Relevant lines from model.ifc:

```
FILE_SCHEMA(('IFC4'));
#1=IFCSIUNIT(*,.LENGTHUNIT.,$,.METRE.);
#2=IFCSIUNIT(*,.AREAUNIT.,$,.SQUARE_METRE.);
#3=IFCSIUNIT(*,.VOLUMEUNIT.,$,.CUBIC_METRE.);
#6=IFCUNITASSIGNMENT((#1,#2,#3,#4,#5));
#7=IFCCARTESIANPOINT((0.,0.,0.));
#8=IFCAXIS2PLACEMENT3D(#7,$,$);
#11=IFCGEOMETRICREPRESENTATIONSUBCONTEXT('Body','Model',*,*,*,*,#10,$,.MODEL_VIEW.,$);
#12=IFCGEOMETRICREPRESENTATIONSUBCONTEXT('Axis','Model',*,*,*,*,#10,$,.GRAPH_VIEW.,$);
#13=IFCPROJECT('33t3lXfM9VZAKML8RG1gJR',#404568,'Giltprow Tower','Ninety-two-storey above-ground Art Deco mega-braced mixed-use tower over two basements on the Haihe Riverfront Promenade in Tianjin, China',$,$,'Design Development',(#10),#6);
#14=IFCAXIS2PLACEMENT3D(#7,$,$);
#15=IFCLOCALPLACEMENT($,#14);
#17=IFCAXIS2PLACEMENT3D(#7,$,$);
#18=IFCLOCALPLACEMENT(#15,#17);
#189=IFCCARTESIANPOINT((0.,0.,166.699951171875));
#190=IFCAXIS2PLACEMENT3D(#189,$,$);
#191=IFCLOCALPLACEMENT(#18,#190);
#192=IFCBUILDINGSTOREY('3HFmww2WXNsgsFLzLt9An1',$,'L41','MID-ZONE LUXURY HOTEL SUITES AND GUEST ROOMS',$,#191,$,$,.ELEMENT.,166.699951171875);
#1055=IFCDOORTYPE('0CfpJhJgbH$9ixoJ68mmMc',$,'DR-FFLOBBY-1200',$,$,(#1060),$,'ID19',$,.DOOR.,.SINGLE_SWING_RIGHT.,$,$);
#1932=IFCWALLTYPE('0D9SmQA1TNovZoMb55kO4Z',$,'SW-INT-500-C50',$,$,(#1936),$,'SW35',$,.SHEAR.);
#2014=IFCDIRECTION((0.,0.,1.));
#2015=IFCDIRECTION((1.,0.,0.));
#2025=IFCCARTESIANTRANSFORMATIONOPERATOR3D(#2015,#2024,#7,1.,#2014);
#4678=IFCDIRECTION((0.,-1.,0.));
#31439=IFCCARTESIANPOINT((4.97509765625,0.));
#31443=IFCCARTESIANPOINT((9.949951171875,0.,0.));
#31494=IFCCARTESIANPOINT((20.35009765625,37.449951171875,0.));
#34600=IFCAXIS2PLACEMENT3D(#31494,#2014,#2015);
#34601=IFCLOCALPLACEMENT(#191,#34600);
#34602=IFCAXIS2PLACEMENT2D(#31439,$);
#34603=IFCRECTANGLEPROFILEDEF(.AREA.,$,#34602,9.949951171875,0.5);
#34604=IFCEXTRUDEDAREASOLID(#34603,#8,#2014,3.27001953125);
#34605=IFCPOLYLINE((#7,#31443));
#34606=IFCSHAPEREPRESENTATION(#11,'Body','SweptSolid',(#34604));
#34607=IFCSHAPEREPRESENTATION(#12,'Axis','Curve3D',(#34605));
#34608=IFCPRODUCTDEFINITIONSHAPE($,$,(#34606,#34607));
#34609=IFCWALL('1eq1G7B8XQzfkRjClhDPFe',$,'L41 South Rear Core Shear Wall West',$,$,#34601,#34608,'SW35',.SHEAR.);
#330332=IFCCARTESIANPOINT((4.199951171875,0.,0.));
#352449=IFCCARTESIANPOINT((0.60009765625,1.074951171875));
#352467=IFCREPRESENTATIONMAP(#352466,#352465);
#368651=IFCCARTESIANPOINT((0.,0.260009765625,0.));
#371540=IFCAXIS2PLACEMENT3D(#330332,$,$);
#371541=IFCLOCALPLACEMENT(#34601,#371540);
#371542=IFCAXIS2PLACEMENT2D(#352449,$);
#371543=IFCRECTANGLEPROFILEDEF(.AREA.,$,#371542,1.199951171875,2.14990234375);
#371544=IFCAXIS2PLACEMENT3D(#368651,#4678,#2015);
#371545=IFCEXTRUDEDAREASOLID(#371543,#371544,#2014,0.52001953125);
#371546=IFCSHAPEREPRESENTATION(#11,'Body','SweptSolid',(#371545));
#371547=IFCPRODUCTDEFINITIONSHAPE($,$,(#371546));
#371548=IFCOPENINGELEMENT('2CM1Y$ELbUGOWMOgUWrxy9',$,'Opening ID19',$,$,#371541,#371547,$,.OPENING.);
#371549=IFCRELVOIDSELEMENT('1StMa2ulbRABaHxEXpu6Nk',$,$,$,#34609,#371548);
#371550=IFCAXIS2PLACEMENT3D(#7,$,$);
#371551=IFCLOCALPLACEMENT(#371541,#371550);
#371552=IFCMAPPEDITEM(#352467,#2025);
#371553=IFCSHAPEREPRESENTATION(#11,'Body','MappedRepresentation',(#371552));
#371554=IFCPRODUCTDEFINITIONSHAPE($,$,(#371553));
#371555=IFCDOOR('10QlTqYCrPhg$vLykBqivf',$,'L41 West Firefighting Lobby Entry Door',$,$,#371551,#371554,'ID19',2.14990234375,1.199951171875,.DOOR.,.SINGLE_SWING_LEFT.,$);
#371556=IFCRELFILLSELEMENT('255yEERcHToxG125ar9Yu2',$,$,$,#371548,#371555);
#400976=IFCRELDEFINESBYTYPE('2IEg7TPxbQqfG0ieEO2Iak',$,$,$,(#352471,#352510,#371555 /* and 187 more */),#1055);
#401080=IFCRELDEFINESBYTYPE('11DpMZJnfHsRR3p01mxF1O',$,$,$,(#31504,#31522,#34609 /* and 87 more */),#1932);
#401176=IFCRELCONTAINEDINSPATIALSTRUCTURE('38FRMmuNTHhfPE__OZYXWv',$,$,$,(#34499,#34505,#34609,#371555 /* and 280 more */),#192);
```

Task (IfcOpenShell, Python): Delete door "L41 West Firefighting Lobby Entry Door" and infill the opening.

```python
import ifcopenshell
import ifcopenshell.api.feature
import ifcopenshell.api.root
import ifcopenshell.geom
import ifcopenshell.util.shape

model = ifcopenshell.open("model.ifc")
settings = ifcopenshell.geom.settings()


def volume(element):
    """Net volume in cubic metres, openings subtracted."""
    shape = ifcopenshell.geom.create_shape(settings, element)
    return ifcopenshell.util.shape.get_volume(shape.geometry)


door = model.by_guid("10QlTqYCrPhg$vLykBqivf")
opening = door.FillsVoids[0].RelatingOpeningElement
wall = opening.VoidsElements[0].RelatingBuildingElement
before = volume(wall)

ifcopenshell.api.root.remove_product(model, product=door)
ifcopenshell.api.feature.remove_feature(model, feature=opening)

after = volume(wall)

print(f"wall volume {before:.3f} -> {after:.3f} m3")

model.write("model_rev.ifc")
```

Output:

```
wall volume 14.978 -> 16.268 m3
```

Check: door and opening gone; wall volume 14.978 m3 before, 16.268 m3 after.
